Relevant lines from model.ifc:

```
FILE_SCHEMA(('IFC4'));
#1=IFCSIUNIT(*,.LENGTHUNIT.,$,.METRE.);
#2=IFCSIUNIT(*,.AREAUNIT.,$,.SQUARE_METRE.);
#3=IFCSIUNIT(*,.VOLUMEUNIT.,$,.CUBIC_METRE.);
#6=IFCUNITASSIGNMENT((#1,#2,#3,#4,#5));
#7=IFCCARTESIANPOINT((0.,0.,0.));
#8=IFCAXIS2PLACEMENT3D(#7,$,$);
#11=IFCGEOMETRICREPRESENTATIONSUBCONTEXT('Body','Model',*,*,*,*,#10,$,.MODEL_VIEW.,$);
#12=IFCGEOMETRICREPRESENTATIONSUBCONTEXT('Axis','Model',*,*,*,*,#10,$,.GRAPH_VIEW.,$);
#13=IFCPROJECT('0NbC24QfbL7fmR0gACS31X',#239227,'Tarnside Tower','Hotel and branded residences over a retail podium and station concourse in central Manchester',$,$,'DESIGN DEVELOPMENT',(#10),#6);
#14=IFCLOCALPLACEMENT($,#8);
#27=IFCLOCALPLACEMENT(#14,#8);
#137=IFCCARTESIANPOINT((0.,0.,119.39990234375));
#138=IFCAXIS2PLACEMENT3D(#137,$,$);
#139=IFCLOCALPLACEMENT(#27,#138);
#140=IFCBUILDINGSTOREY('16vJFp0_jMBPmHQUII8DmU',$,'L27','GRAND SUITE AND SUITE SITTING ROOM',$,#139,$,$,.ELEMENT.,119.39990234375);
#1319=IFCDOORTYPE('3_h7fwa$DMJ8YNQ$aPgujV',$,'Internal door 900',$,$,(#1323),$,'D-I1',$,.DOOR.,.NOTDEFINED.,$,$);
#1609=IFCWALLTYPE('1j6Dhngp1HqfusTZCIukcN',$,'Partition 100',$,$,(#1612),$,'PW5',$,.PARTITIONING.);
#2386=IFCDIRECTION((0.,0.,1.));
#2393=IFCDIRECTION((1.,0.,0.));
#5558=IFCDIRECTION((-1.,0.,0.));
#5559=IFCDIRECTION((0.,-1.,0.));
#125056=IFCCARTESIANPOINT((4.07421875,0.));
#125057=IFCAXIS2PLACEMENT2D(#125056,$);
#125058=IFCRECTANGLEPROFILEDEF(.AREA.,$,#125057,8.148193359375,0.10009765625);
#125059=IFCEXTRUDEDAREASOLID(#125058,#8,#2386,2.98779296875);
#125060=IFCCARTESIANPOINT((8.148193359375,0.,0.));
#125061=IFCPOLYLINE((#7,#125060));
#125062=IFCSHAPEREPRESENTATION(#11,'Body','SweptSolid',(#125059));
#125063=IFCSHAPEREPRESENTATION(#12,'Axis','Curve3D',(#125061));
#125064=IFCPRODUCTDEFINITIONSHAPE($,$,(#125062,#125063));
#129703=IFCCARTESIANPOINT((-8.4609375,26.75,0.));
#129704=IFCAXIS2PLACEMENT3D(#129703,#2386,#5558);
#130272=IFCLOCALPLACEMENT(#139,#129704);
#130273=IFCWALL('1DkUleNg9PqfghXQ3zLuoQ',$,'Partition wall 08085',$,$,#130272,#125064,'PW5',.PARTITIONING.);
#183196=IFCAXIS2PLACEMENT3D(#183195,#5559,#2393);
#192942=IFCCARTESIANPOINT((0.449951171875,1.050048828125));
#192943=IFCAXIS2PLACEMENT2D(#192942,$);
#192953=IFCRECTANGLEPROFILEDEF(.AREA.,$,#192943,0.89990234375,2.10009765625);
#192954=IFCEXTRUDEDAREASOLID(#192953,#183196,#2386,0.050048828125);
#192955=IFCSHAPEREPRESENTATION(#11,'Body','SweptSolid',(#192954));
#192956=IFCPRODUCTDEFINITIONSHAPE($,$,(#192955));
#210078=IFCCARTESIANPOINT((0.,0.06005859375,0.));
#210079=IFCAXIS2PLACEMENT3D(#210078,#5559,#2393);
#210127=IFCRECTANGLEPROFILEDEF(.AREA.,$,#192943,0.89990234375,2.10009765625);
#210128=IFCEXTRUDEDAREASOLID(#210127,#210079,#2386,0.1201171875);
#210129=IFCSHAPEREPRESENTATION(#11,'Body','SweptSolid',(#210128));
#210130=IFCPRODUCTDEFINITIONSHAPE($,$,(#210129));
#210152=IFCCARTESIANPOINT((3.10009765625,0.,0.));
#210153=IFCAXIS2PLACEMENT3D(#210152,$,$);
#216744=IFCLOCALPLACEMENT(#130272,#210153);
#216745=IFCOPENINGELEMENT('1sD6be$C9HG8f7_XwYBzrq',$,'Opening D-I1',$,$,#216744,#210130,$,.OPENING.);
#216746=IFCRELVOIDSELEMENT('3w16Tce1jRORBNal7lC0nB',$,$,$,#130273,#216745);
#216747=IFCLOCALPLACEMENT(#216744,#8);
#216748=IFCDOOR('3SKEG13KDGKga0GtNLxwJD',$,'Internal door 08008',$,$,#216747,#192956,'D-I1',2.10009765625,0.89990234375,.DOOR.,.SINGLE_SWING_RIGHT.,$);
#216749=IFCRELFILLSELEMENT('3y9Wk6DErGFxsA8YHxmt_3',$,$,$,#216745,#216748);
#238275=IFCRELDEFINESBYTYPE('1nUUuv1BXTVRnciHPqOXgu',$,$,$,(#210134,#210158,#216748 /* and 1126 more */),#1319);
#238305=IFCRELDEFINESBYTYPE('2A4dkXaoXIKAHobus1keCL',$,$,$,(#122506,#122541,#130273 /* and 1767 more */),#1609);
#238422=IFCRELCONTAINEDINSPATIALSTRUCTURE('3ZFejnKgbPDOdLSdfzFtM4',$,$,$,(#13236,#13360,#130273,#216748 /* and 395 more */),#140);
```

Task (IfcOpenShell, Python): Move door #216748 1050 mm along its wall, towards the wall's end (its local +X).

```python
import ifcopenshell
import ifcopenshell.api.geometry
import ifcopenshell.util.placement
import ifcopenshell.util.unit

model = ifcopenshell.open("model.ifc")
unit_scale = ifcopenshell.util.unit.calculate_unit_scale(model)

door = model.by_guid("3SKEG13KDGKga0GtNLxwJD")
opening = door.FillsVoids[0].RelatingOpeningElement
wall = opening.VoidsElements[0].RelatingBuildingElement

wall_matrix = ifcopenshell.util.placement.get_local_placement(wall.ObjectPlacement)
shift = wall_matrix[:3, 0] * 1.05 / unit_scale
before = ifcopenshell.util.placement.get_local_placement(door.ObjectPlacement)[:3, 3].copy()

# The door is placed relative to its opening, so it follows when the opening moves.
matrix = ifcopenshell.util.placement.get_local_placement(opening.ObjectPlacement)
matrix[:3, 3] += shift
ifcopenshell.api.geometry.edit_object_placement(
    model, product=opening, matrix=matrix, is_si=False, should_transform_children=True
)

after = ifcopenshell.util.placement.get_local_placement(door.ObjectPlacement)[:3, 3]
print("door moved by", (after - before).round(3) + 0.0)

model.write("model_v2.ifc")
```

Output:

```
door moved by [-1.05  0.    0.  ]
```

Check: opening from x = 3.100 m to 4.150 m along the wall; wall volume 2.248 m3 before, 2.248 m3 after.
